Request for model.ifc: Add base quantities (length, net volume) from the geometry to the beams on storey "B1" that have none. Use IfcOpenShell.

First a look at what the model holds.

```python
import ifcopenshell
import ifcopenshell.util.element
import ifcopenshell.util.unit

model = ifcopenshell.open("model.ifc")
print(model.schema)
for unit_type in ("LENGTHUNIT", "AREAUNIT", "VOLUMEUNIT"):
    print(unit_type, ifcopenshell.util.unit.calculate_unit_scale(model, unit_type))
storey = next(s for s in model.by_type("IfcBuildingStorey") if s.Name == "B1")
beams = [e for e in ifcopenshell.util.element.get_decomposition(storey) if e.is_a("IfcBeam")]
for e in sorted(beams, key=lambda e: e.id()):
    print(e.id(), e.is_a(), e.Name, list(ifcopenshell.util.element.get_psets(e, qtos_only=True)), sep=" | ")
```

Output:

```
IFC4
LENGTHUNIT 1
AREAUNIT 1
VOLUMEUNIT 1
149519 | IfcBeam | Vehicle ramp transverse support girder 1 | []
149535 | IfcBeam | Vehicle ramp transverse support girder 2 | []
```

```python
import ifcopenshell
import ifcopenshell.api.pset
import ifcopenshell.geom
import ifcopenshell.util.element
import ifcopenshell.util.shape
import ifcopenshell.util.unit

model = ifcopenshell.open("model.ifc")
unit_scale = ifcopenshell.util.unit.calculate_unit_scale(model)
volume_scale = ifcopenshell.util.unit.calculate_unit_scale(model, "VOLUMEUNIT")
settings = ifcopenshell.geom.settings()

storey = next(s for s in model.by_type("IfcBuildingStorey") if s.Name == "B1")
beams = [e for e in ifcopenshell.util.element.get_decomposition(storey) if e.is_a("IfcBeam")]

for e in sorted(beams, key=lambda e: e.id()):
    if ifcopenshell.util.element.get_psets(e, qtos_only=True, should_inherit=False):
        continue
    # Geometry comes back in metres, in the element's own axes.
    shape = ifcopenshell.geom.create_shape(settings, e)
    values = {
        "Length": ifcopenshell.util.shape.get_max_xyz(shape.geometry) / unit_scale,
        "NetVolume": ifcopenshell.util.shape.get_volume(shape.geometry) / volume_scale,
    }
    qto = ifcopenshell.api.pset.add_qto(model, product=e, name="Qto_BeamBaseQuantities")
    ifcopenshell.api.pset.edit_qto(model, qto=qto, properties=values)
    print(e.id(), {k: round(v, 3) for k, v in values.items()})

model.write("model-out.ifc")
```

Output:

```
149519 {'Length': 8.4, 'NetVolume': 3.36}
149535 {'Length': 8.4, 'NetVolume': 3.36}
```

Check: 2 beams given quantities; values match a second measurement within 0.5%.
